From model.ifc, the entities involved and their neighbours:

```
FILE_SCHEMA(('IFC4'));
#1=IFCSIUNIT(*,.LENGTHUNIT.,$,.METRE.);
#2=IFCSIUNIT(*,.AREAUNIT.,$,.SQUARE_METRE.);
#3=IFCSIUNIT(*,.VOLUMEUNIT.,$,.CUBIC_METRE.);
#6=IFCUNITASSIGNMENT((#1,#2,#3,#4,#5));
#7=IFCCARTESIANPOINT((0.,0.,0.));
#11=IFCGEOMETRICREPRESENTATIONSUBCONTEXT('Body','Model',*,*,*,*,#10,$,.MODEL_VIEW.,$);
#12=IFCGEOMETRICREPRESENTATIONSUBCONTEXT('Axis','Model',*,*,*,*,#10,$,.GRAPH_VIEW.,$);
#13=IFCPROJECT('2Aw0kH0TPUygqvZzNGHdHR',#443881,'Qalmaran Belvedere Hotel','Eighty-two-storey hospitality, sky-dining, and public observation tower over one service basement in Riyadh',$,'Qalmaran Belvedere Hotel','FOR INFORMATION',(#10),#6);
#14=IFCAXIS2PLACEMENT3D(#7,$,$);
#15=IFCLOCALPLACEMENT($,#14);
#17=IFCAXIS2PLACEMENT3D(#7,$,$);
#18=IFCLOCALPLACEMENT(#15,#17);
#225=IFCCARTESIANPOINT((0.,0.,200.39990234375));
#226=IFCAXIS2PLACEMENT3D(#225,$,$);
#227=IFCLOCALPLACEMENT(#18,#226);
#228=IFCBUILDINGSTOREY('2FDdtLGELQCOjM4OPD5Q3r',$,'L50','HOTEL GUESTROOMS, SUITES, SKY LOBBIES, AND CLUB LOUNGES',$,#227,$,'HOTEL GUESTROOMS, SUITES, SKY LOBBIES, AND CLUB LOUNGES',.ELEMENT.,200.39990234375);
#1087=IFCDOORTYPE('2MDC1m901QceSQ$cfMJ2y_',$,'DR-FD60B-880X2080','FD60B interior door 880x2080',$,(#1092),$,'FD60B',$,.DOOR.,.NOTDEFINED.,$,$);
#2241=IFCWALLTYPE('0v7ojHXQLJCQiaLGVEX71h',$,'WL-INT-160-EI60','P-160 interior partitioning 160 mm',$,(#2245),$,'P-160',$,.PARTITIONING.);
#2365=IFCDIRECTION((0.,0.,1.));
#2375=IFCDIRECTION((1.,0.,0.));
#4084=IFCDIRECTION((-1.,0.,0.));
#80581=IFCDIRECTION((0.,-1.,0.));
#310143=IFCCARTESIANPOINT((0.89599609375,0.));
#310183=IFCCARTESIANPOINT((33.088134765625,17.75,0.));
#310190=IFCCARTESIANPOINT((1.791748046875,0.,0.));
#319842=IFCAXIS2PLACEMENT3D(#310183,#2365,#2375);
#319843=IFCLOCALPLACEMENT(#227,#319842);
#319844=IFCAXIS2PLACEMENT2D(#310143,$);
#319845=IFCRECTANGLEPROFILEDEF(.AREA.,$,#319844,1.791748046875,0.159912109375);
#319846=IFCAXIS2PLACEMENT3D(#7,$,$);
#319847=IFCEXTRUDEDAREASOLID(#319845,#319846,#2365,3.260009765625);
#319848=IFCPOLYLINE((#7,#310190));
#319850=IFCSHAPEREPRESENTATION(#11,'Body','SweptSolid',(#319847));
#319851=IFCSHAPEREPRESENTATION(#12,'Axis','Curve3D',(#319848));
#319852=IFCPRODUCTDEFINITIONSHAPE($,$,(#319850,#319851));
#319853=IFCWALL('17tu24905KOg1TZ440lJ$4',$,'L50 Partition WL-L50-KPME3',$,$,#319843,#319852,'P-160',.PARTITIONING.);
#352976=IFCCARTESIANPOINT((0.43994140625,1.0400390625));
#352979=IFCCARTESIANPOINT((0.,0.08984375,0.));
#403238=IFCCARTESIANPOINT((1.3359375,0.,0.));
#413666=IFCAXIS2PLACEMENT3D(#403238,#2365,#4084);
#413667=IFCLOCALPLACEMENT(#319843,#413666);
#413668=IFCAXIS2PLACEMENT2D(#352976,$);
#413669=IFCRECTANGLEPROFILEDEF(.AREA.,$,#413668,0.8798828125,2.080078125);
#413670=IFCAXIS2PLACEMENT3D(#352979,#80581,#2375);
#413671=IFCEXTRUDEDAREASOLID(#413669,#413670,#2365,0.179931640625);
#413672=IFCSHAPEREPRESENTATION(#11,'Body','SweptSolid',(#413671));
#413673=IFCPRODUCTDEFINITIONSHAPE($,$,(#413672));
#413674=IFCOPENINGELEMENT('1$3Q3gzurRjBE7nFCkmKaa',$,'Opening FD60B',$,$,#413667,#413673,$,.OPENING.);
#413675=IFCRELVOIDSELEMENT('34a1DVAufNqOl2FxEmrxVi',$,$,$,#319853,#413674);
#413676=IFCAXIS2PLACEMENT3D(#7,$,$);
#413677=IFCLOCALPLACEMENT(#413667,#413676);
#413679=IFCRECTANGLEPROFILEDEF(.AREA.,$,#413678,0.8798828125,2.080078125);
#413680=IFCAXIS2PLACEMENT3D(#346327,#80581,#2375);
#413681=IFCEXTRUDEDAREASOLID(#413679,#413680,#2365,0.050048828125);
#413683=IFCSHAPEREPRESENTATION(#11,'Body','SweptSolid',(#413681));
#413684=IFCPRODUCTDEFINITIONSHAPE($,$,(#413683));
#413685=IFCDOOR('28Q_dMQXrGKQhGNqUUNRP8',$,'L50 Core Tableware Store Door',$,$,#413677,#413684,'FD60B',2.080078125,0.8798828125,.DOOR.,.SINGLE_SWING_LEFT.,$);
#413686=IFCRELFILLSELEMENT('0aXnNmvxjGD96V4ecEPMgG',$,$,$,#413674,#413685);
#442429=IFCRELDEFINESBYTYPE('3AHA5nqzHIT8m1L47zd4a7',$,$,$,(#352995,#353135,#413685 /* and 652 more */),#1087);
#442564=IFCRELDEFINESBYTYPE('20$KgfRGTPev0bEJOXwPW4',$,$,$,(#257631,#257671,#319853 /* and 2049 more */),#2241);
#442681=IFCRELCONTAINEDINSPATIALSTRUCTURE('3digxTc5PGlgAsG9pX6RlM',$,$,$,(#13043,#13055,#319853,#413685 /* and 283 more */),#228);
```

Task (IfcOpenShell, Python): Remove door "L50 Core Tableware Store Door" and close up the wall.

```python
import ifcopenshell
import ifcopenshell.api.feature
import ifcopenshell.api.root
import ifcopenshell.geom
import ifcopenshell.util.shape

model = ifcopenshell.open("model.ifc")
settings = ifcopenshell.geom.settings()


def volume(element):
    """Net volume in cubic metres, openings subtracted."""
    shape = ifcopenshell.geom.create_shape(settings, element)
    return ifcopenshell.util.shape.get_volume(shape.geometry)


door = model.by_id(413685)
opening = door.FillsVoids[0].RelatingOpeningElement
wall = opening.VoidsElements[0].RelatingBuildingElement
before = volume(wall)

ifcopenshell.api.root.remove_product(model, product=door)
ifcopenshell.api.feature.remove_feature(model, feature=opening)

after = volume(wall)

print(f"wall volume {before:.3f} -> {after:.3f} m3")

model.write("model-out.ifc")
```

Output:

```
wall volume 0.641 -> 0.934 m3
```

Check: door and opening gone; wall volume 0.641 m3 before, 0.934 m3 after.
